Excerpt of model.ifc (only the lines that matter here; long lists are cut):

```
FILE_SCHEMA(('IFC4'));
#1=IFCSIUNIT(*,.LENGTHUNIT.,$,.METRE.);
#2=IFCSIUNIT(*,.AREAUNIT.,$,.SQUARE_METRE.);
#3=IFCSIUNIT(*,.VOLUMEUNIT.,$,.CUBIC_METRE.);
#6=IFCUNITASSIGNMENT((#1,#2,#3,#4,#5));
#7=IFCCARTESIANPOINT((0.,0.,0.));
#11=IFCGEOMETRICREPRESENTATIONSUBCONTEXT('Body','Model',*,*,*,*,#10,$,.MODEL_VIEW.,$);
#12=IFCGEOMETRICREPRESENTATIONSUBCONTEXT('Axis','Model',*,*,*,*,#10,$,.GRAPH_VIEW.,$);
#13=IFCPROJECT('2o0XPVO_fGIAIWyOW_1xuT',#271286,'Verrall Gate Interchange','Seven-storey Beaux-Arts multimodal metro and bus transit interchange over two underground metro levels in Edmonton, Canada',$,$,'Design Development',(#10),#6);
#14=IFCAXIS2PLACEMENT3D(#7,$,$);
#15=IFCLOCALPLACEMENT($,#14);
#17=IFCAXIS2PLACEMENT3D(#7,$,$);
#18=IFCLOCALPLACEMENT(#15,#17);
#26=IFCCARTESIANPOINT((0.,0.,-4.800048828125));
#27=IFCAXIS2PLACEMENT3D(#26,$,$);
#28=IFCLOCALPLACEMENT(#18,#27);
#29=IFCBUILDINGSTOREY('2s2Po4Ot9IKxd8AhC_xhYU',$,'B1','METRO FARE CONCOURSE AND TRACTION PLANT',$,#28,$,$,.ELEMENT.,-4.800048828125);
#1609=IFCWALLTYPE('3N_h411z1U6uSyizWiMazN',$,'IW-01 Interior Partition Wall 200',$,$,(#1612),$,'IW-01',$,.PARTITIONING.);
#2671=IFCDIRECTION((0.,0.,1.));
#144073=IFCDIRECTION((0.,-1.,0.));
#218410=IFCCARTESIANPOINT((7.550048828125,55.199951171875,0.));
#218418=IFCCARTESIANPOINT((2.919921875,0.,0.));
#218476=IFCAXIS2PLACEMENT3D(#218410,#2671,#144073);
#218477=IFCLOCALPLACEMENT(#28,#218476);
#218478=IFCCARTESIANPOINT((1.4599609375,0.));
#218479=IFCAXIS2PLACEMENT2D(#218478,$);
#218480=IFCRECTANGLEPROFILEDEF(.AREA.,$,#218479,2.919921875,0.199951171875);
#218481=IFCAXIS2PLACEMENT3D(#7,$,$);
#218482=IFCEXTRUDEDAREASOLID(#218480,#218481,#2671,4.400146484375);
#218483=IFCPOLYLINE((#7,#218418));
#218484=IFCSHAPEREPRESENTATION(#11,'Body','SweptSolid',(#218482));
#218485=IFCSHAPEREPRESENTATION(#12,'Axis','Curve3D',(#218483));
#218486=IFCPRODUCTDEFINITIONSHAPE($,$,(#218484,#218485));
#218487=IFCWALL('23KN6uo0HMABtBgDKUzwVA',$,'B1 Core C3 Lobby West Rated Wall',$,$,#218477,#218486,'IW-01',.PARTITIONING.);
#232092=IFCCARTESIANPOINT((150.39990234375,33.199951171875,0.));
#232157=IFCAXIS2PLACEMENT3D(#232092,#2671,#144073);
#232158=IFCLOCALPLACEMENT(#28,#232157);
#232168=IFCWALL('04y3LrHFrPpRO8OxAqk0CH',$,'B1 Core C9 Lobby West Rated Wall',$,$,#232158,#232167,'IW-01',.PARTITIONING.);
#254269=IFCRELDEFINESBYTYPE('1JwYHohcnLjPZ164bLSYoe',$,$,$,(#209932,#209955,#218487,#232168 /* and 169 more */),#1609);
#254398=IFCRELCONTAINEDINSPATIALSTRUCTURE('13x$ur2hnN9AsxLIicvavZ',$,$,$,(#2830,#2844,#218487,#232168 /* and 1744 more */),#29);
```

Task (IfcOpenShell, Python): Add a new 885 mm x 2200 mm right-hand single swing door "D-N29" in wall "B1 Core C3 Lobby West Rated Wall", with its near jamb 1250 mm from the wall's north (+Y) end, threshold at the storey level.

```python
import numpy as np
import ifcopenshell
import ifcopenshell.api.feature
import ifcopenshell.api.geometry
import ifcopenshell.api.root
import ifcopenshell.api.spatial
import ifcopenshell.geom
import ifcopenshell.util.element
import ifcopenshell.util.placement
import ifcopenshell.util.representation
import ifcopenshell.util.shape
import ifcopenshell.util.unit

model = ifcopenshell.open("model.ifc")
unit_scale = ifcopenshell.util.unit.calculate_unit_scale(model)
settings = ifcopenshell.geom.settings()


def volume(element):
    """Net volume in cubic metres, openings subtracted."""
    shape = ifcopenshell.geom.create_shape(settings, element)
    return ifcopenshell.util.shape.get_volume(shape.geometry)


wall = model.by_guid("23KN6uo0HMABtBgDKUzwVA")
storey = ifcopenshell.util.element.get_container(wall, ifc_class="IfcBuildingStorey")
context = ifcopenshell.util.representation.get_context(model, "Model", "Body", "MODEL_VIEW")
before = volume(wall)

width, height, from_end, sill = 0.885, 2.2, 1.25, 0.0  # metres

# The wall runs along its own X axis, and the end named is its -X end.
wall_shape = ifcopenshell.geom.create_shape(settings, wall)
x, y, z = ifcopenshell.util.shape.get_vertices(wall_shape.geometry).T
start = x.min() + from_end
face, thickness = float(y.min()), float(y.max() - y.min())
wall_matrix = ifcopenshell.util.placement.get_local_placement(wall.ObjectPlacement)
level = ifcopenshell.util.placement.get_local_placement(storey.ObjectPlacement)[2, 3]


def in_wall(x, y):
    """Placement at x, y metres in the wall's axes, at sill height."""
    matrix = wall_matrix.copy()
    matrix[:, 3] = wall_matrix @ np.array([x / unit_scale, y / unit_scale, 0.0, 1.0])
    matrix[2, 3] = level + sill / unit_scale
    return matrix


# Opening: a box that overshoots both wall faces by 50 mm.
opening = ifcopenshell.api.root.create_entity(model, ifc_class="IfcOpeningElement", predefined_type="OPENING")
box = ifcopenshell.api.geometry.add_wall_representation(
    model, context=context, length=width, height=height, thickness=thickness + 0.1
)
ifcopenshell.api.geometry.assign_representation(model, product=opening, representation=box)
ifcopenshell.api.geometry.edit_object_placement(model, product=opening, matrix=in_wall(start, face - 0.05), is_si=False)
ifcopenshell.api.feature.add_feature(model, feature=opening, element=wall)

door = ifcopenshell.api.root.create_entity(model, ifc_class="IfcDoor", name="D-N29", predefined_type="DOOR")
door.OverallWidth, door.OverallHeight = width / unit_scale, height / unit_scale
door.OperationType = "SINGLE_SWING_RIGHT"
body = ifcopenshell.api.geometry.add_door_representation(
    model,
    context=context,
    overall_width=door.OverallWidth,
    overall_height=door.OverallHeight,
    operation_type="SINGLE_SWING_RIGHT",
    lining_properties={"LiningDepth": thickness / unit_scale, "ThresholdDepth": thickness / unit_scale},
)
ifcopenshell.api.geometry.assign_representation(model, product=door, representation=body)
ifcopenshell.api.spatial.assign_container(model, products=[door], relating_structure=storey)
ifcopenshell.api.feature.add_filling(model, opening=opening, element=door)

# The lining spans the wall, so the door starts at the wall face.
ifcopenshell.api.geometry.edit_object_placement(model, product=door, matrix=in_wall(start, face), is_si=False)

after = volume(wall)

print(f"wall volume {before:.3f} -> {after:.3f} m3")

model.write("model-out.ifc")
```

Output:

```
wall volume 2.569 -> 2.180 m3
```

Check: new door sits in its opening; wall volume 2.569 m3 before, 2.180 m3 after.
